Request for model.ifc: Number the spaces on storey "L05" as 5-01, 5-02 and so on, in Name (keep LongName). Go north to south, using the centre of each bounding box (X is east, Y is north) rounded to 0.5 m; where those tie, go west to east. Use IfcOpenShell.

First a look at what the model holds.

```python
import ifcopenshell
import ifcopenshell.util.element
import ifcopenshell.util.placement

model = ifcopenshell.open("model.ifc")
print(model.schema)
storey = next(s for s in model.by_type("IfcBuildingStorey") if s.Name == "L05")
spaces = [e for e in ifcopenshell.util.element.get_decomposition(storey) if e.is_a("IfcSpace")]
for e in sorted(spaces, key=lambda e: e.id()):
    origin = ifcopenshell.util.placement.get_local_placement(e.ObjectPlacement)[:3, 3]
    print(e.id(), e.Name, e.LongName, origin.round(2) + 0.0, sep=" | ")
```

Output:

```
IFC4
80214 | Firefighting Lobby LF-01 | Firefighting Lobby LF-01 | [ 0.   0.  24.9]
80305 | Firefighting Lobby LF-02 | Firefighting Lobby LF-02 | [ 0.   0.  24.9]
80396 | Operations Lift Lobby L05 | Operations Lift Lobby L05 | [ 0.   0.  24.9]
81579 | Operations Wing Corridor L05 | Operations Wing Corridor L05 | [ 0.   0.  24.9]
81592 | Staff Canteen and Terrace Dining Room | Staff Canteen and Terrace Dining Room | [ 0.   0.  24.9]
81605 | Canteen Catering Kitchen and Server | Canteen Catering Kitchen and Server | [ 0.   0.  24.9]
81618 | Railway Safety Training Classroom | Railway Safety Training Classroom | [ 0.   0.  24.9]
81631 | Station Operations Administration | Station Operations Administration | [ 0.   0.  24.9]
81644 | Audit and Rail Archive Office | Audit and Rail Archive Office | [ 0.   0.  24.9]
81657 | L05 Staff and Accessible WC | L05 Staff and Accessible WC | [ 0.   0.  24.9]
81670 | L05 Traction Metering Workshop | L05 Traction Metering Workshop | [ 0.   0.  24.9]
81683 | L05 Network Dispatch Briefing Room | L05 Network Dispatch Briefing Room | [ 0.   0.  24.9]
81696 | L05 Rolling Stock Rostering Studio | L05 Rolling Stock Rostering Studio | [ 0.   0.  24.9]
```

```python
import ifcopenshell
import ifcopenshell.geom
import ifcopenshell.util.element
import ifcopenshell.util.shape

model = ifcopenshell.open("model.ifc")
settings = ifcopenshell.geom.settings()
settings.set("use-world-coords", True)


def centre(element):
    shape = ifcopenshell.geom.create_shape(settings, element)
    return ifcopenshell.util.shape.get_bbox_centroid(shape.geometry)


storey = next(s for s in model.by_type("IfcBuildingStorey") if s.Name == "L05")
spaces = [e for e in ifcopenshell.util.element.get_decomposition(storey) if e.is_a("IfcSpace")]

# Insertion points can sit at a corner or the storey origin, so sort by the geometry (in metres).
centres = {e: centre(e) for e in spaces}
spaces.sort(key=lambda e: (-round(centres[e][1] / 0.5), centres[e][0]))

for i, e in enumerate(spaces, start=1):
    number = f"5-{i:02d}"
    e.Name = number
    print(e.id(), number)

model.write("model-out.ifc")
```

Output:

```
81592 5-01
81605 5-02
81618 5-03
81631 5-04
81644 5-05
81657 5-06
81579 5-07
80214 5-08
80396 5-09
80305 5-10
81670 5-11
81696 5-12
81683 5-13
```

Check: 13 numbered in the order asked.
